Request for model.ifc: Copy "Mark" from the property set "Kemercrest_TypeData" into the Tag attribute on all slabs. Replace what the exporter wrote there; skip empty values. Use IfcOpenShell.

First a look at what the model holds.

```python
import ifcopenshell
import ifcopenshell.util.element

model = ifcopenshell.open("model.ifc")
print(model.schema)
slabs = model.by_type("IfcSlab")
print(len(slabs), "slabs")
for e in slabs[:8]:
    source = ifcopenshell.util.element.get_pset(e, "Kemercrest_TypeData", "Mark")
    target = e.Tag
    print(e.id(), repr(source), repr(target), sep=" | ")
```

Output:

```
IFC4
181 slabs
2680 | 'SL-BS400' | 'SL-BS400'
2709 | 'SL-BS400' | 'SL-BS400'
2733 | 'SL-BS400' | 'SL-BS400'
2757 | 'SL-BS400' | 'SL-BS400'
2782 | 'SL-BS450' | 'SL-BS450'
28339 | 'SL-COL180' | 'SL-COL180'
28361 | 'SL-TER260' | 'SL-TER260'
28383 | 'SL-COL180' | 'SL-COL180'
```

```python
import ifcopenshell
import ifcopenshell.util.element

model = ifcopenshell.open("model.ifc")

count = 0
for e in model.by_type("IfcSlab"):
    value = ifcopenshell.util.element.get_pset(e, "Kemercrest_TypeData", "Mark")
    current = e.Tag
    if not value or not value.strip() or current == value:
        continue
    e.Tag = value
    count += 1

print(count, "slabs updated")

model.write("model_updated.ifc")
```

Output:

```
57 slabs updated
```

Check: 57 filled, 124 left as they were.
